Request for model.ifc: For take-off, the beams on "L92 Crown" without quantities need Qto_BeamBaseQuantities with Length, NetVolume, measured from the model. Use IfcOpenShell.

First a look at what the model holds.

```python
import ifcopenshell
import ifcopenshell.util.element
import ifcopenshell.util.unit

model = ifcopenshell.open("model.ifc")
print(model.schema)
for unit_type in ("LENGTHUNIT", "AREAUNIT", "VOLUMEUNIT"):
    print(unit_type, ifcopenshell.util.unit.calculate_unit_scale(model, unit_type))
storey = next(s for s in model.by_type("IfcBuildingStorey") if s.Name == "L92 Crown")
beams = [e for e in ifcopenshell.util.element.get_decomposition(storey) if e.is_a("IfcBeam")]
for e in sorted(beams, key=lambda e: e.id()):
    print(e.id(), e.is_a(), e.Name, list(ifcopenshell.util.element.get_psets(e, qtos_only=True)), sep=" | ")
```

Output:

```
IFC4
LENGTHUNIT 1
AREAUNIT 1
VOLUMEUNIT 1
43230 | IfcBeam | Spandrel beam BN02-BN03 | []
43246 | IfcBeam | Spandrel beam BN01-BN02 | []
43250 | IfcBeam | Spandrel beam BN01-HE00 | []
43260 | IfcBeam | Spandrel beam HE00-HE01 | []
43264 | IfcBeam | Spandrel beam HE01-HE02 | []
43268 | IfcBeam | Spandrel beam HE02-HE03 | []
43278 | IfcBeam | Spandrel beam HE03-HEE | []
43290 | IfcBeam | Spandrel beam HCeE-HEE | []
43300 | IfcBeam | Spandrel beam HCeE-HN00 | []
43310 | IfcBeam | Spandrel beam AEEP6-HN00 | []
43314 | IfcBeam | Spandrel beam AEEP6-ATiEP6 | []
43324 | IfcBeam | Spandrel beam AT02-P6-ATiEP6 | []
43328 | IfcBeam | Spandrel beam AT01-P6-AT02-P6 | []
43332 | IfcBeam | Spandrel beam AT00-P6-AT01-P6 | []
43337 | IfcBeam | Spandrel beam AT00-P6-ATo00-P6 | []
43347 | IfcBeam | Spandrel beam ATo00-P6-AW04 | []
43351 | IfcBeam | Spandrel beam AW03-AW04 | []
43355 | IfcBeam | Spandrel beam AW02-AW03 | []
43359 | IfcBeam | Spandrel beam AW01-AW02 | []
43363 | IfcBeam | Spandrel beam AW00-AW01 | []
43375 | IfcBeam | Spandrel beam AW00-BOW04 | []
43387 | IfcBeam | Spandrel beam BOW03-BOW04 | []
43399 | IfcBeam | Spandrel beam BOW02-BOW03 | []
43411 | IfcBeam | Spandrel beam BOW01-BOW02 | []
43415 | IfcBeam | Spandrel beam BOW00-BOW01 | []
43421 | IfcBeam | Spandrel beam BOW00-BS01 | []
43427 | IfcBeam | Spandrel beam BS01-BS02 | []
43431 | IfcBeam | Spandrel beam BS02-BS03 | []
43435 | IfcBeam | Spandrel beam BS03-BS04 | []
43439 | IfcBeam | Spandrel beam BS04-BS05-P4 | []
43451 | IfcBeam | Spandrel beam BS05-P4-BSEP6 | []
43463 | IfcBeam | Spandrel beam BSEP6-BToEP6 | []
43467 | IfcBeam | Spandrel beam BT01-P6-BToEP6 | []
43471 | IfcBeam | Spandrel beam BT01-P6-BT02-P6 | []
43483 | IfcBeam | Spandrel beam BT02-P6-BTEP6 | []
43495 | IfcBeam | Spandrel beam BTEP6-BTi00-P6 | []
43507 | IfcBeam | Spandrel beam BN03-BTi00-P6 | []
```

```python
import ifcopenshell
import ifcopenshell.api.pset
import ifcopenshell.geom
import ifcopenshell.util.element
import ifcopenshell.util.shape
import ifcopenshell.util.unit

model = ifcopenshell.open("model.ifc")
unit_scale = ifcopenshell.util.unit.calculate_unit_scale(model)
volume_scale = ifcopenshell.util.unit.calculate_unit_scale(model, "VOLUMEUNIT")
settings = ifcopenshell.geom.settings()

storey = next(s for s in model.by_type("IfcBuildingStorey") if s.Name == "L92 Crown")
beams = [e for e in ifcopenshell.util.element.get_decomposition(storey) if e.is_a("IfcBeam")]

for e in sorted(beams, key=lambda e: e.id()):
    if ifcopenshell.util.element.get_psets(e, qtos_only=True, should_inherit=False):
        continue
    # Geometry comes back in metres, in the element's own axes.
    shape = ifcopenshell.geom.create_shape(settings, e)
    values = {
        "Length": ifcopenshell.util.shape.get_max_xyz(shape.geometry) / unit_scale,
        "NetVolume": ifcopenshell.util.shape.get_volume(shape.geometry) / volume_scale,
    }
    qto = ifcopenshell.api.pset.add_qto(model, product=e, name="Qto_BeamBaseQuantities")
    ifcopenshell.api.pset.edit_qto(model, qto=qto, properties=values)
    print(e.id(), {k: round(v, 3) for k, v in values.items()})

model.write("model_updated.ifc")
```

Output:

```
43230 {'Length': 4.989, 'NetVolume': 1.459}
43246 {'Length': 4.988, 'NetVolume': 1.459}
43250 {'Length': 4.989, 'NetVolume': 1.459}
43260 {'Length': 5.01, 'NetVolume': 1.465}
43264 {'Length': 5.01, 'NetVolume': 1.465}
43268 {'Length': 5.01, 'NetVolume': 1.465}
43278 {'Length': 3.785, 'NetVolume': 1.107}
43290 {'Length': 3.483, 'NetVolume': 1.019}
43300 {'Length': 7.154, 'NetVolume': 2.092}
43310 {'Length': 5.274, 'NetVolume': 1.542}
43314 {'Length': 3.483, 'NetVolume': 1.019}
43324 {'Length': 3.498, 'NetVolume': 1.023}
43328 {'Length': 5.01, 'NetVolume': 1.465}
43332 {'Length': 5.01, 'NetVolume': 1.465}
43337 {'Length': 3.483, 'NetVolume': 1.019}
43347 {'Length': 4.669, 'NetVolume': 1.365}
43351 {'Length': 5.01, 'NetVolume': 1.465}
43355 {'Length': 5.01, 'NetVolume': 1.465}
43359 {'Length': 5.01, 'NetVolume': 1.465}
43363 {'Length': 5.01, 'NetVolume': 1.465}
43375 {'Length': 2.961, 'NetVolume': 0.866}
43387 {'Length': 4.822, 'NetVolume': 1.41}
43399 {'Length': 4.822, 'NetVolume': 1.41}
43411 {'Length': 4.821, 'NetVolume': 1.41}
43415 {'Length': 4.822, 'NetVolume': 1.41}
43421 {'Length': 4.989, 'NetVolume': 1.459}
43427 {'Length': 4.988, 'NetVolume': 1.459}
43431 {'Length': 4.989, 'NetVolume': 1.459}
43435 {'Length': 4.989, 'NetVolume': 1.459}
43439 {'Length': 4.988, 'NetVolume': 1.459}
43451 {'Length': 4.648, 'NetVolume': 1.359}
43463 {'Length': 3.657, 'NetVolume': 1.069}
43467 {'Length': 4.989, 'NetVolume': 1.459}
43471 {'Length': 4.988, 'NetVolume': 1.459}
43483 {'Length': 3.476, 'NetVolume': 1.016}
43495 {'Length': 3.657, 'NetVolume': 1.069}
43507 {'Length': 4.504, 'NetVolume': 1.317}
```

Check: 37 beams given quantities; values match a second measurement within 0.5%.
